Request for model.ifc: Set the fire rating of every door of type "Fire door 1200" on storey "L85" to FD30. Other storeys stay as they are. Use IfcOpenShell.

First a look at what the model holds.

```python
import ifcopenshell
import ifcopenshell.util.element

model = ifcopenshell.open("model.ifc")
print(model.schema)
storey = next(s for s in model.by_type("IfcBuildingStorey") if s.Name == "L85")
doors = [e for e in ifcopenshell.util.element.get_decomposition(storey) if e.is_a("IfcDoor")]
seen = {}
for e in doors:
    element_type = ifcopenshell.util.element.get_type(e)
    key = (element_type.Name if element_type != e and element_type else None, ifcopenshell.util.element.get_pset(e, "Pset_DoorCommon", "FireRating"))
    seen[key] = seen.get(key, 0) + 1
for (name, value), count in sorted(seen.items(), key=str):
    print(count, "x", name, "|", value)
```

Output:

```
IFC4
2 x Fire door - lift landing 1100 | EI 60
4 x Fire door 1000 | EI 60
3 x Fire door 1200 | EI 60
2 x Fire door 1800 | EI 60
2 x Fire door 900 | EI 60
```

```python
import ifcopenshell
import ifcopenshell.api.pset
import ifcopenshell.util.element

model = ifcopenshell.open("model.ifc")

storey = next(s for s in model.by_type("IfcBuildingStorey") if s.Name == "L85")
doors = [e for e in ifcopenshell.util.element.get_decomposition(storey) if e.is_a("IfcDoor")]

count = 0
for e in doors:
    element_type = ifcopenshell.util.element.get_type(e)
    if element_type in (None, e) or element_type.Name != "Fire door 1200":
        continue
    found = ifcopenshell.util.element.get_pset(e, "Pset_DoorCommon", should_inherit=False)
    if found:
        pset = model.by_id(found["id"])
        if len(ifcopenshell.util.element.get_elements_by_pset(pset)) > 1:
            pset = ifcopenshell.api.pset.unshare_pset(model, products=[e], pset=pset)[0]
    else:
        pset = ifcopenshell.api.pset.add_pset(model, product=e, name="Pset_DoorCommon")
    ifcopenshell.api.pset.edit_pset(model, pset=pset, properties={"FireRating": "FD30"})
    count += 1

print(count, "doors updated")

model.write("model_v2.ifc")
```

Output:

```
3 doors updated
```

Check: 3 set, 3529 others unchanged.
